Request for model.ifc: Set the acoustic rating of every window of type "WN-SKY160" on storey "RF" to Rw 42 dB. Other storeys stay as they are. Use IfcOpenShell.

First a look at what the model holds.

```python
import ifcopenshell
import ifcopenshell.util.element

model = ifcopenshell.open("model.ifc")
print(model.schema)
storey = next(s for s in model.by_type("IfcBuildingStorey") if s.Name == "RF")
windows = [e for e in ifcopenshell.util.element.get_decomposition(storey) if e.is_a("IfcWindow")]
seen = {}
for e in windows:
    element_type = ifcopenshell.util.element.get_type(e)
    key = (element_type.Name if element_type != e and element_type else None, ifcopenshell.util.element.get_pset(e, "Pset_WindowCommon", "AcousticRating"))
    seen[key] = seen.get(key, 0) + 1
for (name, value), count in sorted(seen.items(), key=str):
    print(count, "x", name, "|", value)
```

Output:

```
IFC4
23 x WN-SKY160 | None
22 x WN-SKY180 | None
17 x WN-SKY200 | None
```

```python
import ifcopenshell
import ifcopenshell.api.pset
import ifcopenshell.util.element

model = ifcopenshell.open("model.ifc")

storey = next(s for s in model.by_type("IfcBuildingStorey") if s.Name == "RF")
windows = [e for e in ifcopenshell.util.element.get_decomposition(storey) if e.is_a("IfcWindow")]

count = 0
for e in windows:
    element_type = ifcopenshell.util.element.get_type(e)
    if element_type in (None, e) or element_type.Name != "WN-SKY160":
        continue
    # add_pset returns the element's existing set when there is one.
    pset = ifcopenshell.api.pset.add_pset(model, product=e, name="Pset_WindowCommon")
    ifcopenshell.api.pset.edit_pset(model, pset=pset, properties={"AcousticRating": "Rw 42 dB"})
    count += 1

print(count, "windows updated")

model.write("model_rev.ifc")
```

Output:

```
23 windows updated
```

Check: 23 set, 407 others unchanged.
